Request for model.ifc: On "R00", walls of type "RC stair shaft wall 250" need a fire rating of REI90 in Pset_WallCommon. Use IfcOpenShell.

First a look at what the model holds.

```python
import ifcopenshell
import ifcopenshell.util.element

model = ifcopenshell.open("model.ifc")
print(model.schema)
storey = next(s for s in model.by_type("IfcBuildingStorey") if s.Name == "R00")
walls = [e for e in ifcopenshell.util.element.get_decomposition(storey) if e.is_a("IfcWall")]
seen = {}
for e in walls:
    element_type = ifcopenshell.util.element.get_type(e)
    key = (element_type.Name if element_type != e and element_type else None, ifcopenshell.util.element.get_pset(e, "Pset_WallCommon", "FireRating"))
    seen[key] = seen.get(key, 0) + 1
for (name, value), count in sorted(seen.items(), key=str):
    print(count, "x", name, "|", value)
```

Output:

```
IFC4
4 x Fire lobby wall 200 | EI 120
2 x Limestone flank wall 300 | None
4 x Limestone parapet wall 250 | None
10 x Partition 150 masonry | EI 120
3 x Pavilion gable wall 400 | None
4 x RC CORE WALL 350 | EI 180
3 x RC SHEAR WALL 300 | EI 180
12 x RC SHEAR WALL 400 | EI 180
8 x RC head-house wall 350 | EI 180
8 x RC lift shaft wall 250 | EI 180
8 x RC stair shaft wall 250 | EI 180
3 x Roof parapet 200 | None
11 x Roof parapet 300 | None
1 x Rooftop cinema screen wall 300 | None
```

```python
import ifcopenshell
import ifcopenshell.api.pset
import ifcopenshell.util.element

model = ifcopenshell.open("model.ifc")

storey = next(s for s in model.by_type("IfcBuildingStorey") if s.Name == "R00")
walls = [e for e in ifcopenshell.util.element.get_decomposition(storey) if e.is_a("IfcWall")]

count = 0
for e in walls:
    element_type = ifcopenshell.util.element.get_type(e)
    if element_type in (None, e) or element_type.Name != "RC stair shaft wall 250":
        continue
    # add_pset returns the element's existing set when there is one.
    pset = ifcopenshell.api.pset.add_pset(model, product=e, name="Pset_WallCommon")
    ifcopenshell.api.pset.edit_pset(model, pset=pset, properties={"FireRating": "REI90"})
    count += 1

print(count, "walls updated")

model.write("model_rev.ifc")
```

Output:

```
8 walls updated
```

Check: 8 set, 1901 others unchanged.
